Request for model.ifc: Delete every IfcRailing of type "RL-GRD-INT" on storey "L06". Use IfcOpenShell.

First a look at what the model holds.

```python
import ifcopenshell
import ifcopenshell.util.element

model = ifcopenshell.open("model.ifc")
print(model.schema)
storey = next(s for s in model.by_type("IfcBuildingStorey") if s.Name == "L06")
railings = [e for e in ifcopenshell.util.element.get_decomposition(storey) if e.is_a("IfcRailing")]
seen = {}
for e in railings:
    element_type = ifcopenshell.util.element.get_type(e)
    name = element_type.Name if element_type not in (None, e) else None
    seen[name] = seen.get(name, 0) + 1
for name, count in sorted(seen.items(), key=str):
    print(count, "x", name)
```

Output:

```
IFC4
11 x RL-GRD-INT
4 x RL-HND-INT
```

```python
import ifcopenshell
import ifcopenshell.api.root
import ifcopenshell.util.element

model = ifcopenshell.open("model.ifc")

storey = next(s for s in model.by_type("IfcBuildingStorey") if s.Name == "L06")
railings = [e for e in ifcopenshell.util.element.get_decomposition(storey) if e.is_a("IfcRailing")]
targets = [e for e in railings if (t := ifcopenshell.util.element.get_type(e)) not in (None, e) and t.Name == "RL-GRD-INT"]

for e in targets:
    ifcopenshell.api.root.remove_product(model, product=e)
print(len(targets), "removed")

model.write("model-out.ifc")
```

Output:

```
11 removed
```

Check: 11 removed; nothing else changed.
